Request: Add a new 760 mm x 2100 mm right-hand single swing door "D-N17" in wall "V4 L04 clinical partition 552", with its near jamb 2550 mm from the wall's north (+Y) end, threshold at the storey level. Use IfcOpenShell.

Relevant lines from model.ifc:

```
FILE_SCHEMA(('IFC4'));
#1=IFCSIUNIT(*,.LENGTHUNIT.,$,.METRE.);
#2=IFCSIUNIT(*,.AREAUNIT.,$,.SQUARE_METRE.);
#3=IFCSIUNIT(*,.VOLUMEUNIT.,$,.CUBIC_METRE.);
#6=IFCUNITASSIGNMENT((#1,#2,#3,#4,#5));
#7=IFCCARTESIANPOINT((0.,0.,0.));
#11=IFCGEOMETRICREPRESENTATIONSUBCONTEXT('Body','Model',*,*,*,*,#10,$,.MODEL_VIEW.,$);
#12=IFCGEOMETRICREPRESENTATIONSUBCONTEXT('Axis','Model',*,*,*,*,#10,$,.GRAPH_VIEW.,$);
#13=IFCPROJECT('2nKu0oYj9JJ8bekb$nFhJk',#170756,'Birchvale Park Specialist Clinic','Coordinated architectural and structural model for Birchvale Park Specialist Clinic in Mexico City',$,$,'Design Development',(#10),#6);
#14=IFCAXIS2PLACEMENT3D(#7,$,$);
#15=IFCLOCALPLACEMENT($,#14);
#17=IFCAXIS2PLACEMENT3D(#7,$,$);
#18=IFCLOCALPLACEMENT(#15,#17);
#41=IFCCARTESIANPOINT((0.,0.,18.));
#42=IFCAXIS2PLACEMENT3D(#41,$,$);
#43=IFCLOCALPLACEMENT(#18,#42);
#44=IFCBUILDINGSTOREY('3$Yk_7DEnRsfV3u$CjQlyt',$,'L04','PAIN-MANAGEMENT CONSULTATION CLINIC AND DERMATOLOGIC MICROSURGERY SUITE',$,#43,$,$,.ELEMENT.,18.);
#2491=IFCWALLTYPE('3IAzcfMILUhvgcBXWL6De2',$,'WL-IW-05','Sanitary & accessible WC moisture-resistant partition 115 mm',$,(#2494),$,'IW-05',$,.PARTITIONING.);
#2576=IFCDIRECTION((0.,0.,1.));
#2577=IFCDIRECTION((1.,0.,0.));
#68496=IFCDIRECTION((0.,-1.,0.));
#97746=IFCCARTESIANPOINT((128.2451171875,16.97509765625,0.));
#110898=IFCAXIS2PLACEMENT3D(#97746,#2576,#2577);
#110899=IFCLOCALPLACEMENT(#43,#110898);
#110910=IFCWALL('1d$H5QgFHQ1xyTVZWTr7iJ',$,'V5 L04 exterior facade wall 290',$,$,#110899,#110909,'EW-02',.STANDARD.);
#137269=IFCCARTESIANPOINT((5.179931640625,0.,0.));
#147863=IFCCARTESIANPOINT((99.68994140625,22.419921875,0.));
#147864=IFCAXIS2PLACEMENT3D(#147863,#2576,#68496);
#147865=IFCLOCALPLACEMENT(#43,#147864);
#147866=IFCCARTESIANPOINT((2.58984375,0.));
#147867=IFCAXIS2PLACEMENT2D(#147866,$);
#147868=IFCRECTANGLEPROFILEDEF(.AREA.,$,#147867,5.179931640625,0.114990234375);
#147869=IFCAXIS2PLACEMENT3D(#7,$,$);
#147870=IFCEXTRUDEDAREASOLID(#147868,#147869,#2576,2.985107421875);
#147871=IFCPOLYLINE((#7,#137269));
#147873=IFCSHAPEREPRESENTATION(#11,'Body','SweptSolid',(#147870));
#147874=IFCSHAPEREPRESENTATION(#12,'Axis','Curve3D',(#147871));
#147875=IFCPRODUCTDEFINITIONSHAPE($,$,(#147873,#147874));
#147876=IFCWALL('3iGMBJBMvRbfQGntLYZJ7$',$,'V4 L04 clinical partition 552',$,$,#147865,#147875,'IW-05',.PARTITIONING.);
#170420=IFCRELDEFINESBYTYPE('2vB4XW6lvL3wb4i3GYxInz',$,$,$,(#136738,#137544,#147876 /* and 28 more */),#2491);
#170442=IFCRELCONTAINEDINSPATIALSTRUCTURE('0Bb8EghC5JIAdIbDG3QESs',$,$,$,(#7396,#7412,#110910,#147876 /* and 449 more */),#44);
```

```python
import numpy as np
import ifcopenshell
import ifcopenshell.api.feature
import ifcopenshell.api.geometry
import ifcopenshell.api.root
import ifcopenshell.api.spatial
import ifcopenshell.geom
import ifcopenshell.util.element
import ifcopenshell.util.placement
import ifcopenshell.util.representation
import ifcopenshell.util.shape
import ifcopenshell.util.unit

model = ifcopenshell.open("model.ifc")
unit_scale = ifcopenshell.util.unit.calculate_unit_scale(model)
settings = ifcopenshell.geom.settings()


def volume(element):
    """Net volume in cubic metres, openings subtracted."""
    shape = ifcopenshell.geom.create_shape(settings, element)
    return ifcopenshell.util.shape.get_volume(shape.geometry)


wall = model.by_id(147876)
storey = ifcopenshell.util.element.get_container(wall, ifc_class="IfcBuildingStorey")
context = ifcopenshell.util.representation.get_context(model, "Model", "Body", "MODEL_VIEW")
before = volume(wall)

width, height, from_end, sill = 0.76, 2.1, 2.55, 0.0  # metres

# The wall runs along its own X axis, and the end named is its -X end.
wall_shape = ifcopenshell.geom.create_shape(settings, wall)
x, y, z = ifcopenshell.util.shape.get_vertices(wall_shape.geometry).T
start = x.min() + from_end
face, thickness = float(y.min()), float(y.max() - y.min())
wall_matrix = ifcopenshell.util.placement.get_local_placement(wall.ObjectPlacement)
level = ifcopenshell.util.placement.get_local_placement(storey.ObjectPlacement)[2, 3]


def in_wall(x, y):
    """Placement at x, y metres in the wall's axes, at sill height."""
    matrix = wall_matrix.copy()
    matrix[:, 3] = wall_matrix @ np.array([x / unit_scale, y / unit_scale, 0.0, 1.0])
    matrix[2, 3] = level + sill / unit_scale
    return matrix


# Opening: a box that overshoots both wall faces by 50 mm.
opening = ifcopenshell.api.root.create_entity(model, ifc_class="IfcOpeningElement", predefined_type="OPENING")
box = ifcopenshell.api.geometry.add_wall_representation(
    model, context=context, length=width, height=height, thickness=thickness + 0.1
)
ifcopenshell.api.geometry.assign_representation(model, product=opening, representation=box)
ifcopenshell.api.geometry.edit_object_placement(model, product=opening, matrix=in_wall(start, face - 0.05), is_si=False)
ifcopenshell.api.feature.add_feature(model, feature=opening, element=wall)

door = ifcopenshell.api.root.create_entity(model, ifc_class="IfcDoor", name="D-N17", predefined_type="DOOR")
door.OverallWidth, door.OverallHeight = width / unit_scale, height / unit_scale
door.OperationType = "SINGLE_SWING_RIGHT"
body = ifcopenshell.api.geometry.add_door_representation(
    model,
    context=context,
    overall_width=door.OverallWidth,
    overall_height=door.OverallHeight,
    operation_type="SINGLE_SWING_RIGHT",
    lining_properties={"LiningDepth": thickness / unit_scale, "ThresholdDepth": thickness / unit_scale},
)
ifcopenshell.api.geometry.assign_representation(model, product=door, representation=body)
ifcopenshell.api.spatial.assign_container(model, products=[door], relating_structure=storey)
ifcopenshell.api.feature.add_filling(model, opening=opening, element=door)

# The lining spans the wall, so the door starts at the wall face.
ifcopenshell.api.geometry.edit_object_placement(model, product=door, matrix=in_wall(start, face), is_si=False)

after = volume(wall)

print(f"wall volume {before:.3f} -> {after:.3f} m3")

model.write("model_updated.ifc")
```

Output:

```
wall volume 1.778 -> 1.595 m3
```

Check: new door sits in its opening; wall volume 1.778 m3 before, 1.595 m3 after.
